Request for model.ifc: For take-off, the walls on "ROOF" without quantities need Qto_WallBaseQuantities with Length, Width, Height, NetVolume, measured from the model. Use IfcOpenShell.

First a look at what the model holds.

```python
import ifcopenshell
import ifcopenshell.util.element
import ifcopenshell.util.unit

model = ifcopenshell.open("model.ifc")
print(model.schema)
for unit_type in ("LENGTHUNIT", "AREAUNIT", "VOLUMEUNIT"):
    print(unit_type, ifcopenshell.util.unit.calculate_unit_scale(model, unit_type))
storey = next(s for s in model.by_type("IfcBuildingStorey") if s.Name == "ROOF")
walls = [e for e in ifcopenshell.util.element.get_decomposition(storey) if e.is_a("IfcWall")]
for e in sorted(walls, key=lambda e: e.id()):
    print(e.id(), e.is_a(), e.Name, list(ifcopenshell.util.element.get_psets(e, qtos_only=True)), sep=" | ")
```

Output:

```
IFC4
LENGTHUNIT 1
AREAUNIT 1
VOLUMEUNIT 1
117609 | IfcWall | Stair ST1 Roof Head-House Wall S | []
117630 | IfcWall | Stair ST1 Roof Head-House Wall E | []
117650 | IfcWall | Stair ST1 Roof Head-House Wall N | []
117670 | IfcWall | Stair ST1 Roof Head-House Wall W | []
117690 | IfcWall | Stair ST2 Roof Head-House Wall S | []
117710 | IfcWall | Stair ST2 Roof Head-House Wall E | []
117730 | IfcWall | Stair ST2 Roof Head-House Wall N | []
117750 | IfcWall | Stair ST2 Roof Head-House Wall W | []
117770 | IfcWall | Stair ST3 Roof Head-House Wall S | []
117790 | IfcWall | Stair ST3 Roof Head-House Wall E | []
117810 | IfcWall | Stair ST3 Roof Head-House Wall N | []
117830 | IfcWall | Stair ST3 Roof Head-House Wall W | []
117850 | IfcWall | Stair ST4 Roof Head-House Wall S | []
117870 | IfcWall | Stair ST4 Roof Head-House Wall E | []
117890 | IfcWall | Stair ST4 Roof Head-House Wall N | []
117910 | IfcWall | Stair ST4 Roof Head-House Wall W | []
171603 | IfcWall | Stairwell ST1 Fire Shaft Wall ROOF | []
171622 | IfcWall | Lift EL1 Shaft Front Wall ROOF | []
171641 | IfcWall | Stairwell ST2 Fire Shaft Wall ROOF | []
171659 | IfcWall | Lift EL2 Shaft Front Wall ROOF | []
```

```python
import ifcopenshell
import ifcopenshell.api.pset
import ifcopenshell.geom
import ifcopenshell.util.element
import ifcopenshell.util.shape
import ifcopenshell.util.unit

model = ifcopenshell.open("model.ifc")
unit_scale = ifcopenshell.util.unit.calculate_unit_scale(model)
volume_scale = ifcopenshell.util.unit.calculate_unit_scale(model, "VOLUMEUNIT")
settings = ifcopenshell.geom.settings()

storey = next(s for s in model.by_type("IfcBuildingStorey") if s.Name == "ROOF")
walls = [e for e in ifcopenshell.util.element.get_decomposition(storey) if e.is_a("IfcWall")]

for e in sorted(walls, key=lambda e: e.id()):
    if ifcopenshell.util.element.get_psets(e, qtos_only=True, should_inherit=False):
        continue
    # Geometry comes back in metres, in the element's own axes.
    shape = ifcopenshell.geom.create_shape(settings, e)
    values = {
        "Length": ifcopenshell.util.shape.get_x(shape.geometry) / unit_scale,
        "Width": ifcopenshell.util.shape.get_y(shape.geometry) / unit_scale,
        "Height": ifcopenshell.util.shape.get_z(shape.geometry) / unit_scale,
        "NetVolume": ifcopenshell.util.shape.get_volume(shape.geometry) / volume_scale,
    }
    qto = ifcopenshell.api.pset.add_qto(model, product=e, name="Qto_WallBaseQuantities")
    ifcopenshell.api.pset.edit_qto(model, qto=qto, properties=values)
    print(e.id(), {k: round(v, 3) for k, v in values.items()})

model.write("model_rev.ifc")
```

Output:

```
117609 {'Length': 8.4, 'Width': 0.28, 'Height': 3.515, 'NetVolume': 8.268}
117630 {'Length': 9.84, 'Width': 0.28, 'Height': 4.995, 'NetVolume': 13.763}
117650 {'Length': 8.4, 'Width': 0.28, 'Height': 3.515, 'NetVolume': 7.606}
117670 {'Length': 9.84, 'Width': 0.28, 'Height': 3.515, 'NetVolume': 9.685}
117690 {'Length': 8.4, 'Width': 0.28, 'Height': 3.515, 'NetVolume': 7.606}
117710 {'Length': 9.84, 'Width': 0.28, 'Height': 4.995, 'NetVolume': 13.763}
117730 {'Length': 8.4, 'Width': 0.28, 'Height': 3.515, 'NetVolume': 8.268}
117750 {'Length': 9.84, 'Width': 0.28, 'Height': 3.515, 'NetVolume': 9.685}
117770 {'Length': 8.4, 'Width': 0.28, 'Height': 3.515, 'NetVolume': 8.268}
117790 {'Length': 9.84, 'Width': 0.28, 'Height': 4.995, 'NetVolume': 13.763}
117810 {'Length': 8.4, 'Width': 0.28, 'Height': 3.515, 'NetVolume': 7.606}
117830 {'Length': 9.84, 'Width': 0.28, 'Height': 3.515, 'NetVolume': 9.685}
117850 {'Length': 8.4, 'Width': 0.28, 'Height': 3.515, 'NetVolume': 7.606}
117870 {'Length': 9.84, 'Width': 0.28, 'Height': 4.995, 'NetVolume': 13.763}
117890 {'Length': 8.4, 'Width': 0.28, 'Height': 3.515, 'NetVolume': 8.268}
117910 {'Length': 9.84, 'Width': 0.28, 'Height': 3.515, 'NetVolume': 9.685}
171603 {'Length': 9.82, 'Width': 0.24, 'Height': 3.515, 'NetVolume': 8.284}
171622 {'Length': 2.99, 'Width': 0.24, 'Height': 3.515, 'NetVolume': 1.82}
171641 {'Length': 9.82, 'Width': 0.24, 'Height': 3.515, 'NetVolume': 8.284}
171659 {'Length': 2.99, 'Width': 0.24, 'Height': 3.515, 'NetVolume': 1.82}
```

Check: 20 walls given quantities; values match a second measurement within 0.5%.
